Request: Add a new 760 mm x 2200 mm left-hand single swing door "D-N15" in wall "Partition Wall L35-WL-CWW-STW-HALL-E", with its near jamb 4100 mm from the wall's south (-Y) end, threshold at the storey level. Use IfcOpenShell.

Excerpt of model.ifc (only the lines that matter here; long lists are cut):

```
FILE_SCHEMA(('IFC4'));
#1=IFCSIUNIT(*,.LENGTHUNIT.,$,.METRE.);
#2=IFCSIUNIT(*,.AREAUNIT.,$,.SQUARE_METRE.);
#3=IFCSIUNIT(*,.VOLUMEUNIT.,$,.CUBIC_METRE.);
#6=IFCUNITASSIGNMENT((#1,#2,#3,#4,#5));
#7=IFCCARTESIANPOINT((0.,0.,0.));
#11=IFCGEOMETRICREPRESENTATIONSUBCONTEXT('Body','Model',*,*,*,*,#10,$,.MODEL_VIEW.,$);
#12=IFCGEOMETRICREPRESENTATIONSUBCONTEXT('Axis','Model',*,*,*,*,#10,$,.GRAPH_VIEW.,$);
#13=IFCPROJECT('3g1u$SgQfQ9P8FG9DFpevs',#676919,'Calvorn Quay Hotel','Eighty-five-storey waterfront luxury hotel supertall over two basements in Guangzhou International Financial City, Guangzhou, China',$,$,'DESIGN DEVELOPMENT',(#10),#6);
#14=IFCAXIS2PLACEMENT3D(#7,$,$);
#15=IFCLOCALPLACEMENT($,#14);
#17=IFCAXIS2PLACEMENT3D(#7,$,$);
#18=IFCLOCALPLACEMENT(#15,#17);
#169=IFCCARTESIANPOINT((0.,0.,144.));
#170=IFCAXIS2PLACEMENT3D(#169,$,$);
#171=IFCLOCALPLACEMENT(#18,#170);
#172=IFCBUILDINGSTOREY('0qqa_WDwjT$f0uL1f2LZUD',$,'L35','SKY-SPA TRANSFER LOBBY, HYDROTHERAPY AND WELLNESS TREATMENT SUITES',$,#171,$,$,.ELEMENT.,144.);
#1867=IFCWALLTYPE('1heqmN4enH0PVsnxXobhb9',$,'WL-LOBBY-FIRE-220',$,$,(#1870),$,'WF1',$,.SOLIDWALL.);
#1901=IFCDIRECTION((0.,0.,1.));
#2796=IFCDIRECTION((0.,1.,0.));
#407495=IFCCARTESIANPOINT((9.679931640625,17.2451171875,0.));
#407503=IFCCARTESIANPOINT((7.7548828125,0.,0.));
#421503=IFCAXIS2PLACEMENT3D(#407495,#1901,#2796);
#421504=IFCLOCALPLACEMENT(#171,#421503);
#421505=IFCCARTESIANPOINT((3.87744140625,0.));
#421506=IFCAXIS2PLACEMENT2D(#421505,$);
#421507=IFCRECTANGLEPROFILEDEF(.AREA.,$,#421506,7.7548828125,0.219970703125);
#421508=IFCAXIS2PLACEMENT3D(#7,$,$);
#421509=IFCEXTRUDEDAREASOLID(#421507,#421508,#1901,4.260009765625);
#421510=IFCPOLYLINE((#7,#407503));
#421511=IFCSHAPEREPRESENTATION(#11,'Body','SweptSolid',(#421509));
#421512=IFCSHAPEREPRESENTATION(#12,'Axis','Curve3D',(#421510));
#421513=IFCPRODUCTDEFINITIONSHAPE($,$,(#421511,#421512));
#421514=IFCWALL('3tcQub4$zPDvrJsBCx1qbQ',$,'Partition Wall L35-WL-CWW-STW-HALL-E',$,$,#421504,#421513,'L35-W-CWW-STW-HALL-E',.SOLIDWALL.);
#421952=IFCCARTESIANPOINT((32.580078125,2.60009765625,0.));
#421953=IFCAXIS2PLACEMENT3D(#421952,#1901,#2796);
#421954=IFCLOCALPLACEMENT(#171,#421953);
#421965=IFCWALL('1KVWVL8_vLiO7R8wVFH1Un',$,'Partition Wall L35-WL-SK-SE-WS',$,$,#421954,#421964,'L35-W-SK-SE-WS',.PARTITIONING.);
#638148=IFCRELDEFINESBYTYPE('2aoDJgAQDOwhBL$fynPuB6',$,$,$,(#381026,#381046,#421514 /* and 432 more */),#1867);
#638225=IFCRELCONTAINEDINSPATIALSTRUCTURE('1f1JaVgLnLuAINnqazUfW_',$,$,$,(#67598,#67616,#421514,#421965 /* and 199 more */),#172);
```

```python
import numpy as np
import ifcopenshell
import ifcopenshell.api.feature
import ifcopenshell.api.geometry
import ifcopenshell.api.root
import ifcopenshell.api.spatial
import ifcopenshell.geom
import ifcopenshell.util.element
import ifcopenshell.util.placement
import ifcopenshell.util.representation
import ifcopenshell.util.shape
import ifcopenshell.util.unit

model = ifcopenshell.open("model.ifc")
unit_scale = ifcopenshell.util.unit.calculate_unit_scale(model)
settings = ifcopenshell.geom.settings()


def volume(element):
    """Net volume in cubic metres, openings subtracted."""
    shape = ifcopenshell.geom.create_shape(settings, element)
    return ifcopenshell.util.shape.get_volume(shape.geometry)


wall = model.by_guid("3tcQub4$zPDvrJsBCx1qbQ")
storey = ifcopenshell.util.element.get_container(wall, ifc_class="IfcBuildingStorey")
context = ifcopenshell.util.representation.get_context(model, "Model", "Body", "MODEL_VIEW")
before = volume(wall)

width, height, from_end, sill = 0.76, 2.2, 4.1, 0.0  # metres

# The wall runs along its own X axis, and the end named is its -X end.
wall_shape = ifcopenshell.geom.create_shape(settings, wall)
x, y, z = ifcopenshell.util.shape.get_vertices(wall_shape.geometry).T
start = x.min() + from_end
face, thickness = float(y.min()), float(y.max() - y.min())
wall_matrix = ifcopenshell.util.placement.get_local_placement(wall.ObjectPlacement)
level = ifcopenshell.util.placement.get_local_placement(storey.ObjectPlacement)[2, 3]


def in_wall(x, y):
    """Placement at x, y metres in the wall's axes, at sill height."""
    matrix = wall_matrix.copy()
    matrix[:, 3] = wall_matrix @ np.array([x / unit_scale, y / unit_scale, 0.0, 1.0])
    matrix[2, 3] = level + sill / unit_scale
    return matrix


# Opening: a box that overshoots both wall faces by 50 mm.
opening = ifcopenshell.api.root.create_entity(model, ifc_class="IfcOpeningElement", predefined_type="OPENING")
box = ifcopenshell.api.geometry.add_wall_representation(
    model, context=context, length=width, height=height, thickness=thickness + 0.1
)
ifcopenshell.api.geometry.assign_representation(model, product=opening, representation=box)
ifcopenshell.api.geometry.edit_object_placement(model, product=opening, matrix=in_wall(start, face - 0.05), is_si=False)
ifcopenshell.api.feature.add_feature(model, feature=opening, element=wall)

door = ifcopenshell.api.root.create_entity(model, ifc_class="IfcDoor", name="D-N15", predefined_type="DOOR")
door.OverallWidth, door.OverallHeight = width / unit_scale, height / unit_scale
door.OperationType = "SINGLE_SWING_LEFT"
body = ifcopenshell.api.geometry.add_door_representation(
    model,
    context=context,
    overall_width=door.OverallWidth,
    overall_height=door.OverallHeight,
    operation_type="SINGLE_SWING_LEFT",
    lining_properties={"LiningDepth": thickness / unit_scale, "ThresholdDepth": thickness / unit_scale},
)
ifcopenshell.api.geometry.assign_representation(model, product=door, representation=body)
ifcopenshell.api.spatial.assign_container(model, products=[door], relating_structure=storey)
ifcopenshell.api.feature.add_filling(model, opening=opening, element=door)

# The lining spans the wall, so the door starts at the wall face.
ifcopenshell.api.geometry.edit_object_placement(model, product=door, matrix=in_wall(start, face), is_si=False)

after = volume(wall)

print(f"wall volume {before:.3f} -> {after:.3f} m3")

model.write("model_v2.ifc")
```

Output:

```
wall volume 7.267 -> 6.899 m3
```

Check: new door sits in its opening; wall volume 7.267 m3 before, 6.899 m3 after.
